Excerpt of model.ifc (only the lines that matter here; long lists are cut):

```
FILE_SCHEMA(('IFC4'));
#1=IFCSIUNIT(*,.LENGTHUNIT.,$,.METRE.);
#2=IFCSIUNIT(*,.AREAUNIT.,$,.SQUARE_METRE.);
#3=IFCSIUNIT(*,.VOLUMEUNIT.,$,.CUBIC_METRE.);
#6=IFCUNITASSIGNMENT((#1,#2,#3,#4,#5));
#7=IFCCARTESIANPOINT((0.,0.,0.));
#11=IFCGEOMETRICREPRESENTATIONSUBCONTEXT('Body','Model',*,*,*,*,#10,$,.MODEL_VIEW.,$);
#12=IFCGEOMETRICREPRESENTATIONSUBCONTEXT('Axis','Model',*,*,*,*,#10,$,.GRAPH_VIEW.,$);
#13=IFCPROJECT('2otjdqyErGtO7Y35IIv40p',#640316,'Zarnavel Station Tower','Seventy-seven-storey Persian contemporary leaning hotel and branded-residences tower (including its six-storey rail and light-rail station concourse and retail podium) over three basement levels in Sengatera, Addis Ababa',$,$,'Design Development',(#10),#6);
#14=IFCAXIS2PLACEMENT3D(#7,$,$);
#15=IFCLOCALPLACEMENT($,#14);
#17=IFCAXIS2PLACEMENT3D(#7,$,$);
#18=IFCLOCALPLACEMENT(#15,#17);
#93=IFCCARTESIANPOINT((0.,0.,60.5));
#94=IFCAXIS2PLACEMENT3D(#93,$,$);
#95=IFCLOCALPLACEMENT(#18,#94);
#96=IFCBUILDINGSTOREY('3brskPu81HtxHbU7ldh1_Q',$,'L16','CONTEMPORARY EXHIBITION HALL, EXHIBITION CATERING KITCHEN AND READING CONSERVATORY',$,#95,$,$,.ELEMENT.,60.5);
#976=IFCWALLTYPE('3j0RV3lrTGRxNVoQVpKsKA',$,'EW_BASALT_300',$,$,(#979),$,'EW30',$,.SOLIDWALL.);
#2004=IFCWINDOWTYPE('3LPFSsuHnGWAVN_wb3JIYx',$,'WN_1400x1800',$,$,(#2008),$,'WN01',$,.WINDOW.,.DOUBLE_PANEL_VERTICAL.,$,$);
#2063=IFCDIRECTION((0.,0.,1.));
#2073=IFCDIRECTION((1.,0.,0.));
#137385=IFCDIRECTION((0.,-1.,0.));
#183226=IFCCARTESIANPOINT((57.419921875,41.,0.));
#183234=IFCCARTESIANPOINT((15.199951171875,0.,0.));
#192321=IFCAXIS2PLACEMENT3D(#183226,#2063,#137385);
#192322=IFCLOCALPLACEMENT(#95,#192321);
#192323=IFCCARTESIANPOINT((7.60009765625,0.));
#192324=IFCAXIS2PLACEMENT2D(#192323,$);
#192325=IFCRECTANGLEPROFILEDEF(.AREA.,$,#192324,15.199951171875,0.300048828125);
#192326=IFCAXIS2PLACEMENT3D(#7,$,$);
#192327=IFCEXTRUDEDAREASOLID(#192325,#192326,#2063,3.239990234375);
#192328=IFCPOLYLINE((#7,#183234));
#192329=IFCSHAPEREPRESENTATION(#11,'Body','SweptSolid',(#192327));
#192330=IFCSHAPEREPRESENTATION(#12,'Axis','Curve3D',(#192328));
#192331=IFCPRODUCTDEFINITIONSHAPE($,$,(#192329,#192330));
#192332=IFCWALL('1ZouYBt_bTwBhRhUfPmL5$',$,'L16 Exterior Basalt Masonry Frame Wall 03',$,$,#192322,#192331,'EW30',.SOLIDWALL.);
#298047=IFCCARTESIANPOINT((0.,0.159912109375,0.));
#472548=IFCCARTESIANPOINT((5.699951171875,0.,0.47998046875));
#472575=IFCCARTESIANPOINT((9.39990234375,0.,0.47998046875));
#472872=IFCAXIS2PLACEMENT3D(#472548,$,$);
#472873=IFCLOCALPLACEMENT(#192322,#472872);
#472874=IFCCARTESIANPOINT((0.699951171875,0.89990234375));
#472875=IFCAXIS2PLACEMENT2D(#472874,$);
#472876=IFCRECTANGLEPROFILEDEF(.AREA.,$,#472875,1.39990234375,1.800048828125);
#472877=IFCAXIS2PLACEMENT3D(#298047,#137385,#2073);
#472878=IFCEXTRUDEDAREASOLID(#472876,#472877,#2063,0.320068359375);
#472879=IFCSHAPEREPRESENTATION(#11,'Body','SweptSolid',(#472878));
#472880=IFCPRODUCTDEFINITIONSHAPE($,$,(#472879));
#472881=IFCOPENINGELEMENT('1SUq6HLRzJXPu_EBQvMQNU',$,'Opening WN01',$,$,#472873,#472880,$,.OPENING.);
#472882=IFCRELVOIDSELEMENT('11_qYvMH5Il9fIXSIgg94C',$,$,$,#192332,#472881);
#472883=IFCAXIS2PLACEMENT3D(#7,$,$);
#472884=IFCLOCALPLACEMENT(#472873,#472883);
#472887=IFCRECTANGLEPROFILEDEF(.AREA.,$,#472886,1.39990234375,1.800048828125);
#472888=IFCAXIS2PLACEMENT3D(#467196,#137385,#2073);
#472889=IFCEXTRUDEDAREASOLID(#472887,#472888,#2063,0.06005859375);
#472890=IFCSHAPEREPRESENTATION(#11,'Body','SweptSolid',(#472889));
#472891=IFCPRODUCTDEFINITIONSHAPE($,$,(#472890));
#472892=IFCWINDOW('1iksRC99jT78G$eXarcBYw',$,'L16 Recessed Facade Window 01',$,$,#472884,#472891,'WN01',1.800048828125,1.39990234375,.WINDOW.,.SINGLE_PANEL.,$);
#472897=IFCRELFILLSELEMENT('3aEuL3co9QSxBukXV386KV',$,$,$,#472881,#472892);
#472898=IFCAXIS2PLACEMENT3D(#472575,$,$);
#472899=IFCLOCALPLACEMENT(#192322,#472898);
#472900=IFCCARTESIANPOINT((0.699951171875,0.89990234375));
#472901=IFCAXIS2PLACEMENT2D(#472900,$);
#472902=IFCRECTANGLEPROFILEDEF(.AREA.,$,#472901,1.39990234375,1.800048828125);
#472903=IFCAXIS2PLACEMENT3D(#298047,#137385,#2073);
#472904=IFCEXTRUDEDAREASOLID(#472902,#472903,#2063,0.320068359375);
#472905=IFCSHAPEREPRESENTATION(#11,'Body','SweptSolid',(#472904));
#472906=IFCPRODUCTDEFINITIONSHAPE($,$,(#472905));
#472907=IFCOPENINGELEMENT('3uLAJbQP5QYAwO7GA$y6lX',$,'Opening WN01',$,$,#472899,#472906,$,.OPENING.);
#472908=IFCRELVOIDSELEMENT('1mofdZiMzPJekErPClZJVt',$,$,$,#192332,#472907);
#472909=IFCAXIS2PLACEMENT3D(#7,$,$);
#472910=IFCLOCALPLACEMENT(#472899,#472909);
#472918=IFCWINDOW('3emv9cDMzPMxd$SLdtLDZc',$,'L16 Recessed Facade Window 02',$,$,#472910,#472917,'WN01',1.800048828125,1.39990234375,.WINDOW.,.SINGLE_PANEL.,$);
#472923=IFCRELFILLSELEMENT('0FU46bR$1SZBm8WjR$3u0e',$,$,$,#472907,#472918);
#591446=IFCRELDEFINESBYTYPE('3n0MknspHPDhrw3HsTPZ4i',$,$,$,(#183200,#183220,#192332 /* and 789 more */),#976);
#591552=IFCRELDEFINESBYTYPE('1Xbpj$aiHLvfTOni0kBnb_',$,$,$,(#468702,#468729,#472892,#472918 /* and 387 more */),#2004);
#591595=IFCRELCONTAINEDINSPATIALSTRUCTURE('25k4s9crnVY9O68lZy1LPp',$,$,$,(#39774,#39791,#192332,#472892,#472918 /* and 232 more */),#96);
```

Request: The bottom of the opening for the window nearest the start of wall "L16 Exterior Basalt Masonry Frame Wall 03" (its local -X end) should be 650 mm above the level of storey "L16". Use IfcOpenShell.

```python
import numpy as np
import ifcopenshell
import ifcopenshell.api.geometry
import ifcopenshell.geom
import ifcopenshell.util.element
import ifcopenshell.util.placement
import ifcopenshell.util.shape
import ifcopenshell.util.unit

model = ifcopenshell.open("model.ifc")
unit_scale = ifcopenshell.util.unit.calculate_unit_scale(model)

window = model.by_guid("1iksRC99jT78G$eXarcBYw")
opening = window.FillsVoids[0].RelatingOpeningElement
storey = ifcopenshell.util.element.get_container(window, ifc_class="IfcBuildingStorey")
level = ifcopenshell.util.placement.get_local_placement(storey.ObjectPlacement)[2, 3]

# The opening's origin need not be at the sill, so measure its lowest point.
shape = ifcopenshell.geom.create_shape(ifcopenshell.geom.settings(), opening)
bottom = ifcopenshell.util.shape.get_shape_bottom_elevation(shape, shape.geometry) / unit_scale
dz = level + 0.65 / unit_scale - bottom

shift = np.array([0.0, 0.0, dz])
# The window is placed relative to its opening, so it follows when the opening moves.
matrix = ifcopenshell.util.placement.get_local_placement(opening.ObjectPlacement)
matrix[:3, 3] += shift
ifcopenshell.api.geometry.edit_object_placement(
    model, product=opening, matrix=matrix, is_si=False, should_transform_children=True
)

print(f"moved by {dz * unit_scale:+.3f} m")

model.write("model-out.ifc")
```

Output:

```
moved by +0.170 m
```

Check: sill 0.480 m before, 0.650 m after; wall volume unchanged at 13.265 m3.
